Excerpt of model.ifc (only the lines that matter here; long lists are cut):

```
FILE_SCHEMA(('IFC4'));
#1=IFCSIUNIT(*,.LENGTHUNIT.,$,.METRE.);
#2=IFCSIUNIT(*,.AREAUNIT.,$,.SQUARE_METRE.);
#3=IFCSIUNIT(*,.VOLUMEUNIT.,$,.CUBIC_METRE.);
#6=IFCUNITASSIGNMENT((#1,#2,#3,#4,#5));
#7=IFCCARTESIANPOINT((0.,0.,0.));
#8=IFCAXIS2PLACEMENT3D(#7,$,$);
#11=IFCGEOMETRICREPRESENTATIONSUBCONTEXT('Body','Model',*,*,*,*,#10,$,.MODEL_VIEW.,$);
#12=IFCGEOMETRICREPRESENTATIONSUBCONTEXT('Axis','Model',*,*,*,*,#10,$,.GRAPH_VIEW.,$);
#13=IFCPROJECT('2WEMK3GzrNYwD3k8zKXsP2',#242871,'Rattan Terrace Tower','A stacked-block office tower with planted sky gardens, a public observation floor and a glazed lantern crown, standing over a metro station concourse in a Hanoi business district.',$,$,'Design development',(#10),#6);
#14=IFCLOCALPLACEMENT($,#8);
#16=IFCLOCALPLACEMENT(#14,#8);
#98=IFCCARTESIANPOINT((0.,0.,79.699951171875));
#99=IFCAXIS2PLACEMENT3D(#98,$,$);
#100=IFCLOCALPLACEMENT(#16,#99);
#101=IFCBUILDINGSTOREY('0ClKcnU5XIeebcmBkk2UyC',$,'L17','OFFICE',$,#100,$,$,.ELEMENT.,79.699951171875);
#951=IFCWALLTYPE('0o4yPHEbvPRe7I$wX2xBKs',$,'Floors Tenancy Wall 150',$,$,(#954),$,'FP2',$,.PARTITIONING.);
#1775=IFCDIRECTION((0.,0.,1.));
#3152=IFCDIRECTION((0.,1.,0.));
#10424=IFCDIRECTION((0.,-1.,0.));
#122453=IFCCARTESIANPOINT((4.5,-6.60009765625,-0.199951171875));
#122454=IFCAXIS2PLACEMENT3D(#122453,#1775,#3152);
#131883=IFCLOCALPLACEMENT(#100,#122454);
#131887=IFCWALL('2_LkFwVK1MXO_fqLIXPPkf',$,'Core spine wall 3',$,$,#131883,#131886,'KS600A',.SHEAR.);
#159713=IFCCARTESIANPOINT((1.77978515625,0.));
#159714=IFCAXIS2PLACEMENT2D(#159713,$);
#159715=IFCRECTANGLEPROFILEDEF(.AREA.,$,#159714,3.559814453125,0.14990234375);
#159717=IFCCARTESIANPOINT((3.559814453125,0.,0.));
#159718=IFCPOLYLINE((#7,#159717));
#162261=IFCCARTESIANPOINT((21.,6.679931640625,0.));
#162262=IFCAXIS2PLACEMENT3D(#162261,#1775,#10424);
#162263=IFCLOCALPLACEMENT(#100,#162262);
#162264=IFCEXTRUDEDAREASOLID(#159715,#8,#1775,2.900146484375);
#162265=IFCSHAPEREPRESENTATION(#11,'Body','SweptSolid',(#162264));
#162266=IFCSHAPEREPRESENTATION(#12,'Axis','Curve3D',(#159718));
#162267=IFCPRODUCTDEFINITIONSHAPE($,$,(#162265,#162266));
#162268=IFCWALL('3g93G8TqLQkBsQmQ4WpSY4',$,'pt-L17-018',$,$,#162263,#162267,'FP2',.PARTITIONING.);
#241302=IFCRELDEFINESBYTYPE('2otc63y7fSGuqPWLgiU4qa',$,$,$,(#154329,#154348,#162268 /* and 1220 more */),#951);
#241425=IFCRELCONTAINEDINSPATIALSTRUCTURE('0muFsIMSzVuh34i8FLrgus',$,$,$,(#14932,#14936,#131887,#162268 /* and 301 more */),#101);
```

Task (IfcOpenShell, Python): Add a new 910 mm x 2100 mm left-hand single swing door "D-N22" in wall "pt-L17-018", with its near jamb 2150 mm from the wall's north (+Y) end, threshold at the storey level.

```python
import numpy as np
import ifcopenshell
import ifcopenshell.api.feature
import ifcopenshell.api.geometry
import ifcopenshell.api.root
import ifcopenshell.api.spatial
import ifcopenshell.geom
import ifcopenshell.util.element
import ifcopenshell.util.placement
import ifcopenshell.util.representation
import ifcopenshell.util.shape
import ifcopenshell.util.unit

model = ifcopenshell.open("model.ifc")
unit_scale = ifcopenshell.util.unit.calculate_unit_scale(model)
settings = ifcopenshell.geom.settings()


def volume(element):
    """Net volume in cubic metres, openings subtracted."""
    shape = ifcopenshell.geom.create_shape(settings, element)
    return ifcopenshell.util.shape.get_volume(shape.geometry)


wall = model.by_guid("3g93G8TqLQkBsQmQ4WpSY4")
storey = ifcopenshell.util.element.get_container(wall, ifc_class="IfcBuildingStorey")
context = ifcopenshell.util.representation.get_context(model, "Model", "Body", "MODEL_VIEW")
before = volume(wall)

width, height, from_end, sill = 0.91, 2.1, 2.15, 0.0  # metres

# The wall runs along its own X axis, and the end named is its -X end.
wall_shape = ifcopenshell.geom.create_shape(settings, wall)
x, y, z = ifcopenshell.util.shape.get_vertices(wall_shape.geometry).T
start = x.min() + from_end
face, thickness = float(y.min()), float(y.max() - y.min())
wall_matrix = ifcopenshell.util.placement.get_local_placement(wall.ObjectPlacement)
level = ifcopenshell.util.placement.get_local_placement(storey.ObjectPlacement)[2, 3]


def in_wall(x, y):
    """Placement at x, y metres in the wall's axes, at sill height."""
    matrix = wall_matrix.copy()
    matrix[:, 3] = wall_matrix @ np.array([x / unit_scale, y / unit_scale, 0.0, 1.0])
    matrix[2, 3] = level + sill / unit_scale
    return matrix


# Opening: a box that overshoots both wall faces by 50 mm.
opening = ifcopenshell.api.root.create_entity(model, ifc_class="IfcOpeningElement", predefined_type="OPENING")
box = ifcopenshell.api.geometry.add_wall_representation(
    model, context=context, length=width, height=height, thickness=thickness + 0.1
)
ifcopenshell.api.geometry.assign_representation(model, product=opening, representation=box)
ifcopenshell.api.geometry.edit_object_placement(model, product=opening, matrix=in_wall(start, face - 0.05), is_si=False)
ifcopenshell.api.feature.add_feature(model, feature=opening, element=wall)

door = ifcopenshell.api.root.create_entity(model, ifc_class="IfcDoor", name="D-N22", predefined_type="DOOR")
door.OverallWidth, door.OverallHeight = width / unit_scale, height / unit_scale
door.OperationType = "SINGLE_SWING_LEFT"
body = ifcopenshell.api.geometry.add_door_representation(
    model,
    context=context,
    overall_width=door.OverallWidth,
    overall_height=door.OverallHeight,
    operation_type="SINGLE_SWING_LEFT",
    lining_properties={"LiningDepth": thickness / unit_scale, "ThresholdDepth": thickness / unit_scale},
)
ifcopenshell.api.geometry.assign_representation(model, product=door, representation=body)
ifcopenshell.api.spatial.assign_container(model, products=[door], relating_structure=storey)
ifcopenshell.api.feature.add_filling(model, opening=opening, element=door)

# The lining spans the wall, so the door starts at the wall face.
ifcopenshell.api.geometry.edit_object_placement(model, product=door, matrix=in_wall(start, face), is_si=False)

after = volume(wall)

print(f"wall volume {before:.3f} -> {after:.3f} m3")

model.write("model_edited.ifc")
```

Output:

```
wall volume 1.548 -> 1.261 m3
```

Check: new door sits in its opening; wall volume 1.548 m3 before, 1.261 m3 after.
